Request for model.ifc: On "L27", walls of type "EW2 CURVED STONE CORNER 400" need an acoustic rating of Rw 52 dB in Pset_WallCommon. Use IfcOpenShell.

First a look at what the model holds.

```python
import ifcopenshell
import ifcopenshell.util.element

model = ifcopenshell.open("model.ifc")
print(model.schema)
storey = next(s for s in model.by_type("IfcBuildingStorey") if s.Name == "L27")
walls = [e for e in ifcopenshell.util.element.get_decomposition(storey) if e.is_a("IfcWall")]
seen = {}
for e in walls:
    element_type = ifcopenshell.util.element.get_type(e)
    key = (element_type.Name if element_type != e and element_type else None, ifcopenshell.util.element.get_pset(e, "Pset_WallCommon", "AcousticRating"))
    seen[key] = seen.get(key, 0) + 1
for (name, value), count in sorted(seen.items(), key=str):
    print(count, "x", name, "|", value)
```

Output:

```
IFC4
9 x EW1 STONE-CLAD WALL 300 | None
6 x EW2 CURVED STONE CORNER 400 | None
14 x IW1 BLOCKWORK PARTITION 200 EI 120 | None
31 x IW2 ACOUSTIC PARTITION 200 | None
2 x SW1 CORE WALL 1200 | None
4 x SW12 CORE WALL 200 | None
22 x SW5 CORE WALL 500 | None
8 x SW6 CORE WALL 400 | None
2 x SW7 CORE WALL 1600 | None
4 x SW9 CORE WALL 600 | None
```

```python
import ifcopenshell
import ifcopenshell.api.pset
import ifcopenshell.util.element

model = ifcopenshell.open("model.ifc")

storey = next(s for s in model.by_type("IfcBuildingStorey") if s.Name == "L27")
walls = [e for e in ifcopenshell.util.element.get_decomposition(storey) if e.is_a("IfcWall")]

count = 0
for e in walls:
    element_type = ifcopenshell.util.element.get_type(e)
    if element_type in (None, e) or element_type.Name != "EW2 CURVED STONE CORNER 400":
        continue
    found = ifcopenshell.util.element.get_pset(e, "Pset_WallCommon", should_inherit=False)
    if found:
        pset = model.by_id(found["id"])
        if len(ifcopenshell.util.element.get_elements_by_pset(pset)) > 1:
            pset = ifcopenshell.api.pset.unshare_pset(model, products=[e], pset=pset)[0]
    else:
        pset = ifcopenshell.api.pset.add_pset(model, product=e, name="Pset_WallCommon")
    ifcopenshell.api.pset.edit_pset(model, pset=pset, properties={"AcousticRating": "Rw 52 dB"})
    count += 1

print(count, "walls updated")

model.write("model_v2.ifc")
```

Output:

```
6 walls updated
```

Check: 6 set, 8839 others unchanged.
